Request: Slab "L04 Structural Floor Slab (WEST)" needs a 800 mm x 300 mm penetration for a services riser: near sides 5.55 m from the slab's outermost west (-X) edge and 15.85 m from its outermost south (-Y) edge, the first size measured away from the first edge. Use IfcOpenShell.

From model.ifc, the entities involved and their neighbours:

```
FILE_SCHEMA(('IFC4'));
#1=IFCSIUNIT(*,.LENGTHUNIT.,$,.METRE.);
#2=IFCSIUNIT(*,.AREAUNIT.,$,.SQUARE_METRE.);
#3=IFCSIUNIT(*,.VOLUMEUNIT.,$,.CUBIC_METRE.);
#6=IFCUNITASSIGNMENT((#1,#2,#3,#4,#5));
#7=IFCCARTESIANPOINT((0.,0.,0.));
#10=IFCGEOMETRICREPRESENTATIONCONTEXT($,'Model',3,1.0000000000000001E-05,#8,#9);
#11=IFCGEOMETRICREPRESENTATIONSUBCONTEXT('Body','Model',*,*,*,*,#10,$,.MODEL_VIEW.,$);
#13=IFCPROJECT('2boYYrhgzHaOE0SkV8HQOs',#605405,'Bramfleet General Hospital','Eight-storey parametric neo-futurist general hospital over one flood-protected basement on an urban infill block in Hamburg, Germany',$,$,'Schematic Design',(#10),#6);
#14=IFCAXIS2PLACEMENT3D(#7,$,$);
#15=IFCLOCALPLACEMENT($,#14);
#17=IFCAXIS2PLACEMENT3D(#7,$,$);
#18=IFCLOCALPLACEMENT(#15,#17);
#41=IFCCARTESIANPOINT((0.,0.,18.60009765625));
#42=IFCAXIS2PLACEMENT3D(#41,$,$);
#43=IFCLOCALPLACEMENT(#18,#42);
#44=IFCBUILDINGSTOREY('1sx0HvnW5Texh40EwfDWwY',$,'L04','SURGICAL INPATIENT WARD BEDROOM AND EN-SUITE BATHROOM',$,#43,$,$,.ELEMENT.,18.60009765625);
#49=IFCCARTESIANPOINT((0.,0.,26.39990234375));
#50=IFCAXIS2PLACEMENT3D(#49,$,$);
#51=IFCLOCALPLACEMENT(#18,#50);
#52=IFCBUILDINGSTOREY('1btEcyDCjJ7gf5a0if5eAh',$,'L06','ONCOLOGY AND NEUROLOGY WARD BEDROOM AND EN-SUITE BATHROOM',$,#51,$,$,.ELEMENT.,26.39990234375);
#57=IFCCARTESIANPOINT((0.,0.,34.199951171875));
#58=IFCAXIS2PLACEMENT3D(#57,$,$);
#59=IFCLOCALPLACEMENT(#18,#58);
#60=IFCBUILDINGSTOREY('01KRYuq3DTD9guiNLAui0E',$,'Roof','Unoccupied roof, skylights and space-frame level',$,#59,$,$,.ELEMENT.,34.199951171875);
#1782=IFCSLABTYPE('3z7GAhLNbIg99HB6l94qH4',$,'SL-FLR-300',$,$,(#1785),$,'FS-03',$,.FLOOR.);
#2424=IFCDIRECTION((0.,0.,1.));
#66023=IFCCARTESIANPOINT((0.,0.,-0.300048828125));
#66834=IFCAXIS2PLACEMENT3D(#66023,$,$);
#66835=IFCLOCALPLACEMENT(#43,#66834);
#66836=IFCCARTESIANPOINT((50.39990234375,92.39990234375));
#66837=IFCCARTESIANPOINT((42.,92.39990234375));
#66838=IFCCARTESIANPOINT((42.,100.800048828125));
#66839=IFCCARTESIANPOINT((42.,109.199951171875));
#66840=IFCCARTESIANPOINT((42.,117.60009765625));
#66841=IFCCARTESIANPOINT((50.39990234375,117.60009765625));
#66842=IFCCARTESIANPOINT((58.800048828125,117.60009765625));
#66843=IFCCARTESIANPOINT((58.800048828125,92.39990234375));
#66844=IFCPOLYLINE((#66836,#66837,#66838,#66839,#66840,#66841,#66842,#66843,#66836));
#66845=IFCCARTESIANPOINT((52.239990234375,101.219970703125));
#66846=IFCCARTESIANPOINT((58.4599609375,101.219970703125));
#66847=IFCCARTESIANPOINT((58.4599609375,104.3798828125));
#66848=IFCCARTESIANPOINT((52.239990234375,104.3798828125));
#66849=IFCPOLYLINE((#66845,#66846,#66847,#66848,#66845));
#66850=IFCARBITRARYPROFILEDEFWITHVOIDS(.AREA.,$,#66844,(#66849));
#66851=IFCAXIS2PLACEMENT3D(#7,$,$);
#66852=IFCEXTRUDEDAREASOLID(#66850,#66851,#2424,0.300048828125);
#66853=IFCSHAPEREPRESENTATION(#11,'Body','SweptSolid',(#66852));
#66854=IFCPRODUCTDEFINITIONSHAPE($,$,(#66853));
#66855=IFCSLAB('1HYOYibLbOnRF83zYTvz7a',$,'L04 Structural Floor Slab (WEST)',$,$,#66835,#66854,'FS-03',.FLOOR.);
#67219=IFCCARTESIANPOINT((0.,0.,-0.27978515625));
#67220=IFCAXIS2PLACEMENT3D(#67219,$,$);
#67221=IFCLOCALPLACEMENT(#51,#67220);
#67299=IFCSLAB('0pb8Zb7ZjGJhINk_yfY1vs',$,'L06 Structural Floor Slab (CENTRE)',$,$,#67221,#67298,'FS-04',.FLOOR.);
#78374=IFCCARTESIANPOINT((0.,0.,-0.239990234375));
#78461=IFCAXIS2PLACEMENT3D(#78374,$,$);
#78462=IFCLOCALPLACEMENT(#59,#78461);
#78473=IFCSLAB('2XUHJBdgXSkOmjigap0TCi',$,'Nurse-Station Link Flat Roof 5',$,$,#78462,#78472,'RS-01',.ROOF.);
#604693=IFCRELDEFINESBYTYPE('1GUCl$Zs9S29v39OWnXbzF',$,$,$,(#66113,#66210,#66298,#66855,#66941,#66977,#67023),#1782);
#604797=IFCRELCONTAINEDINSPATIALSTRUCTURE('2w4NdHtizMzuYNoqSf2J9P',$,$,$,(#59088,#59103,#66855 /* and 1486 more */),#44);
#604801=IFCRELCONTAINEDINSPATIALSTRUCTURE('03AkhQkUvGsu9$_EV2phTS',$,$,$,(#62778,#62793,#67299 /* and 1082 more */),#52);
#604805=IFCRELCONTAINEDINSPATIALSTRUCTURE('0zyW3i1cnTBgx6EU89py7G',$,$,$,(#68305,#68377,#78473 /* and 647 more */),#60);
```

```python
import numpy as np
import ifcopenshell
import ifcopenshell.api.feature
import ifcopenshell.api.geometry
import ifcopenshell.api.root
import ifcopenshell.geom
import ifcopenshell.util.placement
import ifcopenshell.util.representation
import ifcopenshell.util.shape
import ifcopenshell.util.unit

model = ifcopenshell.open("model.ifc")
unit_scale = ifcopenshell.util.unit.calculate_unit_scale(model)
settings = ifcopenshell.geom.settings()


def volume(element):
    """Net volume in cubic metres, openings subtracted."""
    shape = ifcopenshell.geom.create_shape(settings, element)
    return ifcopenshell.util.shape.get_volume(shape.geometry)


slab = model.by_guid("1HYOYibLbOnRF83zYTvz7a")
before = volume(slab)

# Extent in the slab's own axes, in metres. The edges named are its -X and -Y sides.
slab_shape = ifcopenshell.geom.create_shape(settings, slab)
vertices = ifcopenshell.util.shape.get_vertices(slab_shape.geometry)
x_min, y_min, bottom = vertices.min(axis=0)
top = vertices[:, 2].max()

opening = ifcopenshell.api.root.create_entity(model, ifc_class="IfcOpeningElement", name="Services riser opening", predefined_type="OPENING")
context = ifcopenshell.util.representation.get_context(model, "Model", "Body", "MODEL_VIEW")
width, depth = 0.8, 0.3
outline = [(0.0, 0.0), (width, 0.0), (width, depth), (0.0, depth), (0.0, 0.0)]
# Overshoot both faces by 50 mm so the cut is clean.
shape = ifcopenshell.api.geometry.add_slab_representation(
    model, context=context, depth=top - bottom + 0.1, polyline=outline
)
ifcopenshell.api.geometry.assign_representation(model, product=opening, representation=shape)

matrix = ifcopenshell.util.placement.get_local_placement(slab.ObjectPlacement)
matrix[:, 3] = matrix @ np.append(np.array([x_min + 5.55, y_min + 15.85, bottom - 0.05]) / unit_scale, 1.0)
ifcopenshell.api.geometry.edit_object_placement(model, product=opening, matrix=matrix, is_si=False)
ifcopenshell.api.feature.add_feature(model, feature=opening, element=slab)

after = volume(slab)

print(f"slab volume {before:.3f} -> {after:.3f} m3")

model.write("model_v2.ifc")
```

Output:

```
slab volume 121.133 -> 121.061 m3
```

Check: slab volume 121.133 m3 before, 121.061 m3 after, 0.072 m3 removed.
